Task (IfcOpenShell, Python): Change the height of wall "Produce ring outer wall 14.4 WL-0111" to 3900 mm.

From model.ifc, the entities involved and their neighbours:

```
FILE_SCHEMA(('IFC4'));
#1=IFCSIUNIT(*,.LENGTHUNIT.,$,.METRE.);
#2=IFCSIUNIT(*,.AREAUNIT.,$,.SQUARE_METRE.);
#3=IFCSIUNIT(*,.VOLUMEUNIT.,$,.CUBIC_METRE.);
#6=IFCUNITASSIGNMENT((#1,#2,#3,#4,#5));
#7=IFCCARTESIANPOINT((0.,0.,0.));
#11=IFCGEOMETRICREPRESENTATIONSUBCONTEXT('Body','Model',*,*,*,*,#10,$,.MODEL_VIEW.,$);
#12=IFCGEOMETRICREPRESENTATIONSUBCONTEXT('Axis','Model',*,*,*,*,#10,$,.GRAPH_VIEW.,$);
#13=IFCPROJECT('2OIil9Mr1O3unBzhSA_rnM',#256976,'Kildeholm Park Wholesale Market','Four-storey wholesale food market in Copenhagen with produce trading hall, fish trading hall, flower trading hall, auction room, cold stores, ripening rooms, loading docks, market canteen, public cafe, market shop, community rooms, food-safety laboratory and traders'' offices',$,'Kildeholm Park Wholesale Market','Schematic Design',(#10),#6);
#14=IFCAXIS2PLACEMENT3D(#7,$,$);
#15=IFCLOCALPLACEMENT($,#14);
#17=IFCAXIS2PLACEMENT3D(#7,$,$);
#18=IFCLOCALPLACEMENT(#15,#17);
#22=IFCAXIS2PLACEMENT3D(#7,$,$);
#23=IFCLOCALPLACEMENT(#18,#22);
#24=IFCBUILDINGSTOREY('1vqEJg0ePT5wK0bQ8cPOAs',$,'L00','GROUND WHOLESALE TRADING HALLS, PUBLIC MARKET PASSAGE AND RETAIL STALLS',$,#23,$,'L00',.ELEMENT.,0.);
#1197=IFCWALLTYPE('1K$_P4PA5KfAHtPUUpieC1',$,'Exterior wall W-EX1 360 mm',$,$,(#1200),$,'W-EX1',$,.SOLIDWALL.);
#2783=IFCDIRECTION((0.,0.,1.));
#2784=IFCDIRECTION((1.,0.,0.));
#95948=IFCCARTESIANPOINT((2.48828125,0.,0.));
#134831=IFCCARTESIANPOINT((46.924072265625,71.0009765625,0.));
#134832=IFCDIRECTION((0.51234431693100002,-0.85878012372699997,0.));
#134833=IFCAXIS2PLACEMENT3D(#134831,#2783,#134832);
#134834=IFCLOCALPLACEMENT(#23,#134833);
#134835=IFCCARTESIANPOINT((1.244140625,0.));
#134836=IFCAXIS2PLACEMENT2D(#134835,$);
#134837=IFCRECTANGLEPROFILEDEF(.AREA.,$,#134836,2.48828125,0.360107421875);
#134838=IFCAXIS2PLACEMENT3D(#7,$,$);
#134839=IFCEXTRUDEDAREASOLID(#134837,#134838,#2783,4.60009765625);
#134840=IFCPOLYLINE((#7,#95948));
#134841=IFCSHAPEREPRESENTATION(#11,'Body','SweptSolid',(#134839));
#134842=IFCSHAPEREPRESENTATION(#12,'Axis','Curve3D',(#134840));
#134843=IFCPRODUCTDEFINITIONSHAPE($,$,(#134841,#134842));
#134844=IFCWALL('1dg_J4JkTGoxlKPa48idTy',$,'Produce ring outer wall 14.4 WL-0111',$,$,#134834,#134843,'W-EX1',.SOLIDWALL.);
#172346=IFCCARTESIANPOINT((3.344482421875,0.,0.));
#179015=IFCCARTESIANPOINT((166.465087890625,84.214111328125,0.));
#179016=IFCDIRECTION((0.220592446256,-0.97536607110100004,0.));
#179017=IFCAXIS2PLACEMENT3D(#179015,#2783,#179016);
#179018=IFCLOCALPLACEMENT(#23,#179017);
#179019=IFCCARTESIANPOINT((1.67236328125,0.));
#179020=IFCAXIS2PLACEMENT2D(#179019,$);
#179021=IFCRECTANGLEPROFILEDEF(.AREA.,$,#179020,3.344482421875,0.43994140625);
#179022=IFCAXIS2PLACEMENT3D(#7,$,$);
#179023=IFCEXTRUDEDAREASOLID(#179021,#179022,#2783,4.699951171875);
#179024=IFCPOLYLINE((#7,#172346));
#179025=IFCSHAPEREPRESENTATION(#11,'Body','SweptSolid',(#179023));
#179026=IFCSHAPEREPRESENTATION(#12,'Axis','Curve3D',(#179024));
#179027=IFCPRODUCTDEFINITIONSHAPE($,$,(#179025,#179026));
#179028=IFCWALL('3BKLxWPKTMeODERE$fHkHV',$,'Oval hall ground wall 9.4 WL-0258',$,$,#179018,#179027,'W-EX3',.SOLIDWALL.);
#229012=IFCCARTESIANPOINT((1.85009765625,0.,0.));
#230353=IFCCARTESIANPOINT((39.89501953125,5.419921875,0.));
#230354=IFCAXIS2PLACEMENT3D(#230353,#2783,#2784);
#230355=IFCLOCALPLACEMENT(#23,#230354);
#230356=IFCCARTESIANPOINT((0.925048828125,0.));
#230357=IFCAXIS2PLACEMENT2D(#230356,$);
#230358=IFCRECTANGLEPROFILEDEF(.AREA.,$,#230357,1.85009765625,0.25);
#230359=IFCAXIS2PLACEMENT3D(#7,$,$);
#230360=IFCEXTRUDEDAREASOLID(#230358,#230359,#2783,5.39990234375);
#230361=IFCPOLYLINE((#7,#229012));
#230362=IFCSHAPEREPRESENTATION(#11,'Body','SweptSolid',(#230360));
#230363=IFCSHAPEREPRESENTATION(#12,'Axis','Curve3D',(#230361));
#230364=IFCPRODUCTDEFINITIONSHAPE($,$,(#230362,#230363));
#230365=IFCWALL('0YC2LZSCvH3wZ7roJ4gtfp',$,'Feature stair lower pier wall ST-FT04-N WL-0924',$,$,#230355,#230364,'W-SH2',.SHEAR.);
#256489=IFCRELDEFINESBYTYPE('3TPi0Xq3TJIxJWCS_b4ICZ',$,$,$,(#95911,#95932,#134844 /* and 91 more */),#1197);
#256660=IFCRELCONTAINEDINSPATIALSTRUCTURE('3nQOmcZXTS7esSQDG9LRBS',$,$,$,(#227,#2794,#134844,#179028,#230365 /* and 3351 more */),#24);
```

```python
import ifcopenshell
import ifcopenshell.geom
import ifcopenshell.util.representation
import ifcopenshell.util.shape

model = ifcopenshell.open("model.ifc")
settings = ifcopenshell.geom.settings()


def volume(element):
    """Net volume in cubic metres, openings subtracted."""
    shape = ifcopenshell.geom.create_shape(settings, element)
    return ifcopenshell.util.shape.get_volume(shape.geometry)


wall = model.by_guid("1dg_J4JkTGoxlKPa48idTy")
before = volume(wall)

body = ifcopenshell.util.representation.get_representation(wall, "Model", "Body")
solid = body.Items[0]
old_height = solid.Depth
solid.Depth = 3.9
after = volume(wall)

print(f"height {old_height:g} -> {solid.Depth:g}, volume {before:.3f} -> {after:.3f} m3")

model.write("model_rev.ifc")
```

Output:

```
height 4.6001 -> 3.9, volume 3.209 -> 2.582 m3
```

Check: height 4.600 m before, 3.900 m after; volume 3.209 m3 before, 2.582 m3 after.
